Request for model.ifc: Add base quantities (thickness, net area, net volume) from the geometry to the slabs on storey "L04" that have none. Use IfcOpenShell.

First a look at what the model holds.

```python
import ifcopenshell
import ifcopenshell.util.element
import ifcopenshell.util.unit

model = ifcopenshell.open("model.ifc")
print(model.schema)
for unit_type in ("LENGTHUNIT", "AREAUNIT", "VOLUMEUNIT"):
    print(unit_type, ifcopenshell.util.unit.calculate_unit_scale(model, unit_type))
storey = next(s for s in model.by_type("IfcBuildingStorey") if s.Name == "L04")
slabs = [e for e in ifcopenshell.util.element.get_decomposition(storey) if e.is_a("IfcSlab")]
for e in sorted(slabs, key=lambda e: e.id()):
    print(e.id(), e.is_a(), e.Name, list(ifcopenshell.util.element.get_psets(e, qtos_only=True)), sep=" | ")
```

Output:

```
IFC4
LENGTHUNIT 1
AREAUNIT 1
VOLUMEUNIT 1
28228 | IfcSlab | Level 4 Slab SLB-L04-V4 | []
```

```python
import ifcopenshell
import ifcopenshell.api.pset
import ifcopenshell.geom
import ifcopenshell.util.element
import ifcopenshell.util.shape
import ifcopenshell.util.unit

model = ifcopenshell.open("model.ifc")
unit_scale = ifcopenshell.util.unit.calculate_unit_scale(model)
area_scale = ifcopenshell.util.unit.calculate_unit_scale(model, "AREAUNIT")
volume_scale = ifcopenshell.util.unit.calculate_unit_scale(model, "VOLUMEUNIT")
settings = ifcopenshell.geom.settings()

storey = next(s for s in model.by_type("IfcBuildingStorey") if s.Name == "L04")
slabs = [e for e in ifcopenshell.util.element.get_decomposition(storey) if e.is_a("IfcSlab")]

for e in sorted(slabs, key=lambda e: e.id()):
    if ifcopenshell.util.element.get_psets(e, qtos_only=True, should_inherit=False):
        continue
    # Geometry comes back in metres, in the element's own axes.
    shape = ifcopenshell.geom.create_shape(settings, e)
    values = {
        "Width": ifcopenshell.util.shape.get_z(shape.geometry) / unit_scale,
        "NetArea": ifcopenshell.util.shape.get_footprint_area(shape.geometry) / area_scale,
        "NetVolume": ifcopenshell.util.shape.get_volume(shape.geometry) / volume_scale,
    }
    qto = ifcopenshell.api.pset.add_qto(model, product=e, name="Qto_SlabBaseQuantities")
    ifcopenshell.api.pset.edit_qto(model, qto=qto, properties=values)
    print(e.id(), {k: round(v, 3) for k, v in values.items()})

model.write("model_rev.ifc")
```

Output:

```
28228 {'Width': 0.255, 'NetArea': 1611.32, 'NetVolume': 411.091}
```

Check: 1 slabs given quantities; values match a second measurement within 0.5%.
